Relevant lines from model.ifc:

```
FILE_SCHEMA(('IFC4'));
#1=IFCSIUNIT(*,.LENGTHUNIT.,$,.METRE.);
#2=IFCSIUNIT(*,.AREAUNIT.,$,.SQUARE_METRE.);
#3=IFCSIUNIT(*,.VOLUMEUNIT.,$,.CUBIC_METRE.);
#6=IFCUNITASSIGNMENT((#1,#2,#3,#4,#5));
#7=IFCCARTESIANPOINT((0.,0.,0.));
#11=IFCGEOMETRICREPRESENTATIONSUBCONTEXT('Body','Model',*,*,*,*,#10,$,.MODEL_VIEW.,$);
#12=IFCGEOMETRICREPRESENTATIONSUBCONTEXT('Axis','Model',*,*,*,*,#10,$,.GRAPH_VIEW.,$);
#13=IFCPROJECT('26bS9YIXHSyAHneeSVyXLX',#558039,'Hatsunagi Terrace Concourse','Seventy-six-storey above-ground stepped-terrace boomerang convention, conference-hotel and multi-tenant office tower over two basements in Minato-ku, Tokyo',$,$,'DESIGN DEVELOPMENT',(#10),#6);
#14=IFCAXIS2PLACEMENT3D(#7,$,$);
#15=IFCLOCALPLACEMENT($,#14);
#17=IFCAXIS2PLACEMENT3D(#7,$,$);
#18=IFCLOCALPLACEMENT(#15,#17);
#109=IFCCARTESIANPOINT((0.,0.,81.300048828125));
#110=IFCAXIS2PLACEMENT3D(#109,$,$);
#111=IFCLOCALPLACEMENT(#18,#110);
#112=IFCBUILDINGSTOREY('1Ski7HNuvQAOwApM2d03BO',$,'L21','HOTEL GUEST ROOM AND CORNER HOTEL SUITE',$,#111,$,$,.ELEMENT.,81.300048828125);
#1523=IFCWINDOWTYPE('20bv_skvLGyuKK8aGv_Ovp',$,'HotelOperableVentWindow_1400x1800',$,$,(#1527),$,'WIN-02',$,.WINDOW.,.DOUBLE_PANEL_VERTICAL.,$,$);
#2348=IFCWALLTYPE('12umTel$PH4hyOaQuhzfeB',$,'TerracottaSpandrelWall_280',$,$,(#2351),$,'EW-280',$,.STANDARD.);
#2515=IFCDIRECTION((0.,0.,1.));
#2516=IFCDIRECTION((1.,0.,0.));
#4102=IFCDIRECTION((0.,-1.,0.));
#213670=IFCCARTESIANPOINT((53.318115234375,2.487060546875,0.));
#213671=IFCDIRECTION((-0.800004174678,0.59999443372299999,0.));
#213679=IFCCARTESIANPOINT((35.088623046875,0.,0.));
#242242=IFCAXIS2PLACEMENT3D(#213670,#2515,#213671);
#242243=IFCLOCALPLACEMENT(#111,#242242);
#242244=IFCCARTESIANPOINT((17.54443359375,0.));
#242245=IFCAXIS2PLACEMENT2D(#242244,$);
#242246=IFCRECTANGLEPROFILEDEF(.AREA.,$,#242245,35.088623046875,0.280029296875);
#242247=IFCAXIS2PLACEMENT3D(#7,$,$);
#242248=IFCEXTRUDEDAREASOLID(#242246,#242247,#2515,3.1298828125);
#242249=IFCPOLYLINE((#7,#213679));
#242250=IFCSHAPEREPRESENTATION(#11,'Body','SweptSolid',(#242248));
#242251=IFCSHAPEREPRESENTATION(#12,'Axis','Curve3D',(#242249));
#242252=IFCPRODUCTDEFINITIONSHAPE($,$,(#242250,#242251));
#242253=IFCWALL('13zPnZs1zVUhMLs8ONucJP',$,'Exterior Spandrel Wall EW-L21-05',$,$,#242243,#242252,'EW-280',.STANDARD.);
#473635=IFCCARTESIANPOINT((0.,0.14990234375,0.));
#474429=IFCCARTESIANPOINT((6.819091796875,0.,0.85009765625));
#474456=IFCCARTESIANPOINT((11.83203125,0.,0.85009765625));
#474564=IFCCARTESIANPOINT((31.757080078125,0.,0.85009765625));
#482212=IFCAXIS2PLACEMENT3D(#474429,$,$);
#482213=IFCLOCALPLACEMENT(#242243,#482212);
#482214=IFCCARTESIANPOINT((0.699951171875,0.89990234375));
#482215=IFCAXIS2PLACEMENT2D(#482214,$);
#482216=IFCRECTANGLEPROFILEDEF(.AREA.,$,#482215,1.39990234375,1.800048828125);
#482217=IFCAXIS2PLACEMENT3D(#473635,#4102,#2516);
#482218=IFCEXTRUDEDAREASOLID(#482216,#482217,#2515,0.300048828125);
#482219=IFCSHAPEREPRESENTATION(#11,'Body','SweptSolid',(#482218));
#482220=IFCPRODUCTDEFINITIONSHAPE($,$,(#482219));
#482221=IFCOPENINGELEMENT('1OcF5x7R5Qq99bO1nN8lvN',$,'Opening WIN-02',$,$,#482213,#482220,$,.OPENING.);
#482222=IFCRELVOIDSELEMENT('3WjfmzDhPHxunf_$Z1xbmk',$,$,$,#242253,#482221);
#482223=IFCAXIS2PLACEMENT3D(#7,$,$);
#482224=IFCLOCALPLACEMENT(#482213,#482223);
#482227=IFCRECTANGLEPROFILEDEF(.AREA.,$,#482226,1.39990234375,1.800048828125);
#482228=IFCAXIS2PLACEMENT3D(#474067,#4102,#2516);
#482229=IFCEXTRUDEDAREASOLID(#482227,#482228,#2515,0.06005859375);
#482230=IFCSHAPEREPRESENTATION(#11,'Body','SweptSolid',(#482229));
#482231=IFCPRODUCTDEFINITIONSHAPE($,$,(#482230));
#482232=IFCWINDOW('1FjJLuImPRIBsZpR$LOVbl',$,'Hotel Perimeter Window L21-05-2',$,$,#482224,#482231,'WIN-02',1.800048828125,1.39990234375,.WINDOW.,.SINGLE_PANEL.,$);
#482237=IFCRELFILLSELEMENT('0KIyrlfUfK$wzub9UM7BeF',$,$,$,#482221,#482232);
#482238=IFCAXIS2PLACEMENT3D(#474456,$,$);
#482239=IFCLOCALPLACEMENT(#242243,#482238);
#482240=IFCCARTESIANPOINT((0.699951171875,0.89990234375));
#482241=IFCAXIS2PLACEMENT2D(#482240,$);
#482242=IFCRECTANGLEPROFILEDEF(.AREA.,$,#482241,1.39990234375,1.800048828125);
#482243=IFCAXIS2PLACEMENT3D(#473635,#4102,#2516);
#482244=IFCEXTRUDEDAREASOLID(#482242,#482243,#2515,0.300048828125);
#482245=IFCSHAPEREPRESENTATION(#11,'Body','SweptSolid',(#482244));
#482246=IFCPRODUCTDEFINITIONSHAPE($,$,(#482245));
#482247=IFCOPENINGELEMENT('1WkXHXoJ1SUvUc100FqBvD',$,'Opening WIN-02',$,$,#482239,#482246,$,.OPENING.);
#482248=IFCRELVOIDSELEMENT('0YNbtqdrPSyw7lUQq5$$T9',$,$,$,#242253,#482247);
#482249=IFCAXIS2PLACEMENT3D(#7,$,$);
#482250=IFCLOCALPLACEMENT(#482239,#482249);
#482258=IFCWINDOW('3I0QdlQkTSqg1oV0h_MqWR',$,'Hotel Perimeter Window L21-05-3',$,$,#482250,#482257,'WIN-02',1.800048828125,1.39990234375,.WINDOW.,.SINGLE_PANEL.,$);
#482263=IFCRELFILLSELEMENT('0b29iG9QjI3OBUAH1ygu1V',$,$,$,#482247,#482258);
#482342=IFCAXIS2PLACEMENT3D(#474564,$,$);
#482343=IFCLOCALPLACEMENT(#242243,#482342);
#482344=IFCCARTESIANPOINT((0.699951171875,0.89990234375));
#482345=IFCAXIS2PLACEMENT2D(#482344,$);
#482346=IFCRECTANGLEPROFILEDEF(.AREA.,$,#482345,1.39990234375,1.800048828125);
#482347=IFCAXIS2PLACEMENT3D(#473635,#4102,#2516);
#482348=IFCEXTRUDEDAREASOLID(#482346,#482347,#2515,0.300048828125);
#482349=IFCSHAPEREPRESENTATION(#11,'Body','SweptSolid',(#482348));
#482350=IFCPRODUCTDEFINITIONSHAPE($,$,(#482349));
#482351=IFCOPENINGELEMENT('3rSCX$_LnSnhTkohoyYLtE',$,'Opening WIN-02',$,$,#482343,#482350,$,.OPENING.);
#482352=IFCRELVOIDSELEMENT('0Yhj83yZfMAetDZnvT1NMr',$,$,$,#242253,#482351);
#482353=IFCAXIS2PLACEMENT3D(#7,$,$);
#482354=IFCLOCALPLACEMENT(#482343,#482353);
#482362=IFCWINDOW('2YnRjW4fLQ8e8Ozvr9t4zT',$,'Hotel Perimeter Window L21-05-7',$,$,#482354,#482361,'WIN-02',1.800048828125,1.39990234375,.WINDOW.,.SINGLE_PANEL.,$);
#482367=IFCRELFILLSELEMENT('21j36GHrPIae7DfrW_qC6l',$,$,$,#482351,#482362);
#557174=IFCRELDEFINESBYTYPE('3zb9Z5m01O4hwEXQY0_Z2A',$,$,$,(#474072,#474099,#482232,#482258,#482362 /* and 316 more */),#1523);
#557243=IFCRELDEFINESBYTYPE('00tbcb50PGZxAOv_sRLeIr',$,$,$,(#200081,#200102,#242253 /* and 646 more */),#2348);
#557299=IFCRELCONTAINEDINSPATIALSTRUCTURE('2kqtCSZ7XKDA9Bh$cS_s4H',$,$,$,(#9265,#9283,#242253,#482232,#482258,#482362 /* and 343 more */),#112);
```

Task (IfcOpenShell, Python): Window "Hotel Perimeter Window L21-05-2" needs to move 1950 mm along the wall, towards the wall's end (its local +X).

```python
import ifcopenshell
import ifcopenshell.api.geometry
import ifcopenshell.util.placement

model = ifcopenshell.open("model.ifc")

window = model.by_guid("1FjJLuImPRIBsZpR$LOVbl")
opening = window.FillsVoids[0].RelatingOpeningElement
wall = opening.VoidsElements[0].RelatingBuildingElement

wall_matrix = ifcopenshell.util.placement.get_local_placement(wall.ObjectPlacement)
shift = wall_matrix[:3, 0] * 1.95
before = ifcopenshell.util.placement.get_local_placement(window.ObjectPlacement)[:3, 3].copy()

# The window is placed relative to its opening, so it follows when the opening moves.
matrix = ifcopenshell.util.placement.get_local_placement(opening.ObjectPlacement)
matrix[:3, 3] += shift
ifcopenshell.api.geometry.edit_object_placement(
    model, product=opening, matrix=matrix, is_si=False, should_transform_children=True
)

after = ifcopenshell.util.placement.get_local_placement(window.ObjectPlacement)[:3, 3]
print("window moved by", (after - before).round(3) + 0.0)

model.write("model-out.ifc")
```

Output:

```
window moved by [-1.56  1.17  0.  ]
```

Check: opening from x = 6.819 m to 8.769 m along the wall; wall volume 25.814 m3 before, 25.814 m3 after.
